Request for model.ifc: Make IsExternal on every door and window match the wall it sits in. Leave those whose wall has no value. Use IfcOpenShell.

First a look at what the model holds.

```python
import ifcopenshell
import ifcopenshell.util.element

model = ifcopenshell.open("model.ifc")
print(model.schema)
seen = {}
for e in model.by_type("IfcDoor") + model.by_type("IfcWindow"):
    if not e.FillsVoids:
        continue
    host = e.FillsVoids[0].RelatingOpeningElement.VoidsElements[0].RelatingBuildingElement
    own = ifcopenshell.util.element.get_pset(e, f"Pset_{e.is_a()[3:].removesuffix('StandardCase')}Common", "IsExternal")
    wall = ifcopenshell.util.element.get_pset(host, "Pset_WallCommon", "IsExternal")
    seen[e.is_a(), own, wall] = seen.get((e.is_a(), own, wall), 0) + 1
for (cls, own, wall), count in sorted(seen.items(), key=str):
    print(count, cls, "IsExternal:", own, "| host wall:", wall)
```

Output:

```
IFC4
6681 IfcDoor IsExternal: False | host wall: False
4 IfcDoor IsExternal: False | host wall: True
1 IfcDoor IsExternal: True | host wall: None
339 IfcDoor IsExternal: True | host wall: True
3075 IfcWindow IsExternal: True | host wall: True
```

```python
import ifcopenshell
import ifcopenshell.api.pset
import ifcopenshell.util.element

model = ifcopenshell.open("model.ifc")

count = 0
for ifc_class, pset_name in (("IfcDoor", "Pset_DoorCommon"), ("IfcWindow", "Pset_WindowCommon")):
    for e in model.by_type(ifc_class):
        if not e.FillsVoids:
            continue
        host = e.FillsVoids[0].RelatingOpeningElement.VoidsElements[0].RelatingBuildingElement
        external = ifcopenshell.util.element.get_pset(host, "Pset_WallCommon", "IsExternal")
        if external is None or ifcopenshell.util.element.get_pset(e, pset_name, "IsExternal") == external:
            continue
        found = ifcopenshell.util.element.get_pset(e, pset_name, should_inherit=False)
        if found:
            pset = model.by_id(found["id"])
            if len(ifcopenshell.util.element.get_elements_by_pset(pset)) > 1:
                pset = ifcopenshell.api.pset.unshare_pset(model, products=[e], pset=pset)[0]
        else:
            pset = ifcopenshell.api.pset.add_pset(model, product=e, name=pset_name)
        ifcopenshell.api.pset.edit_pset(model, pset=pset, properties={"IsExternal": external})
        count += 1

print(count, "updated")

model.write("model_v2.ifc")
```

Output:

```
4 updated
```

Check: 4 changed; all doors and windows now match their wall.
